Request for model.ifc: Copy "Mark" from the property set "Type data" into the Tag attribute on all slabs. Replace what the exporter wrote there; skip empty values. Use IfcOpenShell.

First a look at what the model holds.

```python
import ifcopenshell
import ifcopenshell.util.element

model = ifcopenshell.open("model.ifc")
print(model.schema)
slabs = model.by_type("IfcSlab")
print(len(slabs), "slabs")
for e in slabs[:8]:
    source = ifcopenshell.util.element.get_pset(e, "Type data", "Mark")
    target = e.Tag
    print(e.id(), repr(source), repr(target), sep=" | ")
```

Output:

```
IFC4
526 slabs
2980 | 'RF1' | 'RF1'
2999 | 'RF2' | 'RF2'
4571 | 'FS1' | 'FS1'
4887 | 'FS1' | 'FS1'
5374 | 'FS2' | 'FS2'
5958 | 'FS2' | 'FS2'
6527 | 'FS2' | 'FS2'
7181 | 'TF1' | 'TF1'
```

```python
import ifcopenshell
import ifcopenshell.util.element

model = ifcopenshell.open("model.ifc")

count = 0
for e in model.by_type("IfcSlab"):
    value = ifcopenshell.util.element.get_pset(e, "Type data", "Mark")
    current = e.Tag
    if not value or not value.strip() or current == value:
        continue
    e.Tag = value
    count += 1

print(count, "slabs updated")

model.write("model_rev.ifc")
```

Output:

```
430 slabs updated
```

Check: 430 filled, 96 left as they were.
